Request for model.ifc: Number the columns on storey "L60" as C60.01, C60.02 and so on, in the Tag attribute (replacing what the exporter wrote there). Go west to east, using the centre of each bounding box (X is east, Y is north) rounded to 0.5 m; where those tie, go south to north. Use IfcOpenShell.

First a look at what the model holds.

```python
import ifcopenshell
import ifcopenshell.util.element
import ifcopenshell.util.placement

model = ifcopenshell.open("model.ifc")
print(model.schema)
storey = next(s for s in model.by_type("IfcBuildingStorey") if s.Name == "L60")
columns = [e for e in ifcopenshell.util.element.get_decomposition(storey) if e.is_a("IfcColumn")]
for e in sorted(columns, key=lambda e: e.id()):
    origin = ifcopenshell.util.placement.get_local_placement(e.ObjectPlacement)[:3, 3]
    print(e.id(), e.Tag, e.Name, origin.round(2) + 0.0, sep=" | ")
```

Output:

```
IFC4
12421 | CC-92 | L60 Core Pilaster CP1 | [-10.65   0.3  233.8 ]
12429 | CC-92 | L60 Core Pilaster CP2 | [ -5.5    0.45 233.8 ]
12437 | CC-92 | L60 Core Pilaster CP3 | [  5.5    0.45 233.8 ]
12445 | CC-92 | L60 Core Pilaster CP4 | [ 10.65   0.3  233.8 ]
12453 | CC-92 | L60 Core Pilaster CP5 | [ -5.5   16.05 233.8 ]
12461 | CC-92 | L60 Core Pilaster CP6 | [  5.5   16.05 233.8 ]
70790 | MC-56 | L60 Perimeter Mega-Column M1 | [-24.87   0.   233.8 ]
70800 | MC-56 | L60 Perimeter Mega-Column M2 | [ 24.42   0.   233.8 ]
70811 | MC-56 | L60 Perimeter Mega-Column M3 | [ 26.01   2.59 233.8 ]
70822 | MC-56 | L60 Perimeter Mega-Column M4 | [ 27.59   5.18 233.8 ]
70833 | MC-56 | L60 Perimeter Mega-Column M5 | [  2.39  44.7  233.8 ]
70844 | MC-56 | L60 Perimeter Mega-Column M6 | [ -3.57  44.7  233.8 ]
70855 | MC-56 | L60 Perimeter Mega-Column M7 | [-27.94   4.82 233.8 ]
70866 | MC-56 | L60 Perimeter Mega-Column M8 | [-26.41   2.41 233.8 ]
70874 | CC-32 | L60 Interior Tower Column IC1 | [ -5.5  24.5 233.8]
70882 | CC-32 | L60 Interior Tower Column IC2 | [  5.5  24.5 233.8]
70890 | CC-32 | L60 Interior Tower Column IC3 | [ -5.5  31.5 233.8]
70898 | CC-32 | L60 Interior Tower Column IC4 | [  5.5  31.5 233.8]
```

```python
import ifcopenshell
import ifcopenshell.geom
import ifcopenshell.util.element
import ifcopenshell.util.shape

model = ifcopenshell.open("model.ifc")
settings = ifcopenshell.geom.settings()
settings.set("use-world-coords", True)


def centre(element):
    shape = ifcopenshell.geom.create_shape(settings, element)
    return ifcopenshell.util.shape.get_bbox_centroid(shape.geometry)


storey = next(s for s in model.by_type("IfcBuildingStorey") if s.Name == "L60")
columns = [e for e in ifcopenshell.util.element.get_decomposition(storey) if e.is_a("IfcColumn")]

# Insertion points can sit at a corner or the storey origin, so sort by the geometry (in metres).
centres = {e: centre(e) for e in columns}
columns.sort(key=lambda e: (round(centres[e][0] / 0.5), centres[e][1]))

for i, e in enumerate(columns, start=1):
    number = f"C60.{i:02d}"
    e.Tag = number
    print(e.id(), number)

model.write("model_edited.ifc")
```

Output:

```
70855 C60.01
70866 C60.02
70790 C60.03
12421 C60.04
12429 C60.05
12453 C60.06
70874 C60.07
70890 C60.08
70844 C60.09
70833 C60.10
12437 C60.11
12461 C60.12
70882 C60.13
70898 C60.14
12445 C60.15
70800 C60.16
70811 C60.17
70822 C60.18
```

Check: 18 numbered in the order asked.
